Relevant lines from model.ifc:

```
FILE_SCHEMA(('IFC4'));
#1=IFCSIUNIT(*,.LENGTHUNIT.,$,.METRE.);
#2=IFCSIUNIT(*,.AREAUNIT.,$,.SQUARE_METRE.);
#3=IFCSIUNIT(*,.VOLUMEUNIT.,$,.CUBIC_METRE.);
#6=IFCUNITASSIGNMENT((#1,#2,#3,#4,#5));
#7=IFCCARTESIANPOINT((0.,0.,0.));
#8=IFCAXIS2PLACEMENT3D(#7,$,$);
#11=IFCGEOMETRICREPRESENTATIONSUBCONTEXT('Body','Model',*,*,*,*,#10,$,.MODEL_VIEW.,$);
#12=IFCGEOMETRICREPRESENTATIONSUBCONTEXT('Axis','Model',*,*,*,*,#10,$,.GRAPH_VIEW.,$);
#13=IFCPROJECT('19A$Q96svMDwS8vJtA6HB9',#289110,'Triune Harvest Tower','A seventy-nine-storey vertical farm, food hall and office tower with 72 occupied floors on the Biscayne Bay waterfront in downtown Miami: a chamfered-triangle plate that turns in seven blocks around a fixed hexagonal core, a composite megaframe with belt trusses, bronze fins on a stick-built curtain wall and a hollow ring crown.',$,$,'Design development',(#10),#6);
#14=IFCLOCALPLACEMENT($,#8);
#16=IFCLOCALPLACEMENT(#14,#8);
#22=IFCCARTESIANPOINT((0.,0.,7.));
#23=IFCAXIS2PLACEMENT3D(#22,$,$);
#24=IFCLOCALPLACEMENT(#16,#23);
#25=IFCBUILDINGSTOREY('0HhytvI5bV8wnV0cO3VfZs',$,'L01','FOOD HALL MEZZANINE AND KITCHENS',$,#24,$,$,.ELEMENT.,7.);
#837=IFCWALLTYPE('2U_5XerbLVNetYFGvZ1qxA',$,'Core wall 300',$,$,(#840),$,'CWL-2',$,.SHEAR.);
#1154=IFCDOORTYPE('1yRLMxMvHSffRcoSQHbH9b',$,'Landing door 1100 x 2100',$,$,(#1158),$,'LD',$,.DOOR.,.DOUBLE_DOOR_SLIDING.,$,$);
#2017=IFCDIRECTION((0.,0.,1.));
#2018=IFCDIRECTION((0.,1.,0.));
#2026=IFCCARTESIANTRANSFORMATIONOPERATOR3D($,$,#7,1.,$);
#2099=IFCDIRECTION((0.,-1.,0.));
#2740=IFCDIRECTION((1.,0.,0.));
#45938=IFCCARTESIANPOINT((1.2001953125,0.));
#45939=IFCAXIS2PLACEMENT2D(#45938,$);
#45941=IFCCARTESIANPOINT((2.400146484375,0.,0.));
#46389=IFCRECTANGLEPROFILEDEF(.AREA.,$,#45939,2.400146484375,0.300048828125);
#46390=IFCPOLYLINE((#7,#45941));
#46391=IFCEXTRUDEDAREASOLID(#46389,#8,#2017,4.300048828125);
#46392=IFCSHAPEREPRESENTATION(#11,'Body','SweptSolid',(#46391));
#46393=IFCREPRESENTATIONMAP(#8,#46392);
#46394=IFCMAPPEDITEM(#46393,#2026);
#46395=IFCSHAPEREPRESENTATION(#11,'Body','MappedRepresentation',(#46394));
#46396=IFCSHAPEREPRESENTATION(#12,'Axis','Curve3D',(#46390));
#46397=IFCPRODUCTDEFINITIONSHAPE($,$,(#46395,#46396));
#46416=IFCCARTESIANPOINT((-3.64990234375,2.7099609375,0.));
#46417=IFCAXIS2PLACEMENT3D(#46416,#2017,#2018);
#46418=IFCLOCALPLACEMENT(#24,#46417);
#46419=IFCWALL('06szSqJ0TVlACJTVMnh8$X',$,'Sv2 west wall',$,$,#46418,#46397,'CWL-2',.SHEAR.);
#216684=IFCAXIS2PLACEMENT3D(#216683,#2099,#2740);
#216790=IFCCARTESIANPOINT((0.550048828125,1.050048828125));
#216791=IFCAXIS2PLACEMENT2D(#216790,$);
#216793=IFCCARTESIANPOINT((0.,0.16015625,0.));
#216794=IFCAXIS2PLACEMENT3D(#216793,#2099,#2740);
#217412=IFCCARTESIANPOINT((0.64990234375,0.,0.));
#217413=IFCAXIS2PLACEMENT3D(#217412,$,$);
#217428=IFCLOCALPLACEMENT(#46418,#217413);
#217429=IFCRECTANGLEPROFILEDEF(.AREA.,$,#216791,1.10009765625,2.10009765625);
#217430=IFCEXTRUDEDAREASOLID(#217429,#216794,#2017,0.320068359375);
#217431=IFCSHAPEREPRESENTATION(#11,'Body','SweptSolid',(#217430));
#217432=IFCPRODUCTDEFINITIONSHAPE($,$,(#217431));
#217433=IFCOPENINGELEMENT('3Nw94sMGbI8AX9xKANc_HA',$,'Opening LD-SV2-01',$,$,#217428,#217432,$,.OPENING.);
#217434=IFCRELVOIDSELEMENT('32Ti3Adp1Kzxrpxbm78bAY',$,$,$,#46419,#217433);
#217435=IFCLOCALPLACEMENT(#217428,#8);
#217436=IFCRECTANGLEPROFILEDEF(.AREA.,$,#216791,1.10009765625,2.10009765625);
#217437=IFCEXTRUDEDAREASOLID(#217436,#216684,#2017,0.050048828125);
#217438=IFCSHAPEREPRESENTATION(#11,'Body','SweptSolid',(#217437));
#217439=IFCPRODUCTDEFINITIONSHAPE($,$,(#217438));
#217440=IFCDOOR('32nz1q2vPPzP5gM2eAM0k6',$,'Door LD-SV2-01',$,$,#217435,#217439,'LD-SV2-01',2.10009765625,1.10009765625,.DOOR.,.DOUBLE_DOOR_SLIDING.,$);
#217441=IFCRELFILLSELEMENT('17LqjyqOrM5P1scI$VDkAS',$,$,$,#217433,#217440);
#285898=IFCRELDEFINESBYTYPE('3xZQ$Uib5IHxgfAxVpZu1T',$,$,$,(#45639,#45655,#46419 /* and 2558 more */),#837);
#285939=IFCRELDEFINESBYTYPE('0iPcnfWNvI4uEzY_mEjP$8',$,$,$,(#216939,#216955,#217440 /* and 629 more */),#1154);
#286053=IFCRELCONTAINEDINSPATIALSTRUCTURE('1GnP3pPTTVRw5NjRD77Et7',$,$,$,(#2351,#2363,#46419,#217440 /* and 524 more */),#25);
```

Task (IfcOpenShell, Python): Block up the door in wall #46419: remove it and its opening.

```python
import ifcopenshell
import ifcopenshell.api.feature
import ifcopenshell.api.root
import ifcopenshell.geom
import ifcopenshell.util.shape

model = ifcopenshell.open("model.ifc")
settings = ifcopenshell.geom.settings()


def volume(element):
    """Net volume in cubic metres, openings subtracted."""
    shape = ifcopenshell.geom.create_shape(settings, element)
    return ifcopenshell.util.shape.get_volume(shape.geometry)


door = model.by_id(217440)
opening = door.FillsVoids[0].RelatingOpeningElement
wall = opening.VoidsElements[0].RelatingBuildingElement
before = volume(wall)

ifcopenshell.api.root.remove_product(model, product=door)
ifcopenshell.api.feature.remove_feature(model, feature=opening)

after = volume(wall)

print(f"wall volume {before:.3f} -> {after:.3f} m3")

model.write("model_v2.ifc")
```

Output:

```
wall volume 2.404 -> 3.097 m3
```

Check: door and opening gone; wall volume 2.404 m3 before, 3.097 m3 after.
